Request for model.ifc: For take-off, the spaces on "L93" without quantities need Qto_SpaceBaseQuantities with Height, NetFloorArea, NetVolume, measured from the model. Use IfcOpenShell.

First a look at what the model holds.

```python
import ifcopenshell
import ifcopenshell.util.element
import ifcopenshell.util.unit

model = ifcopenshell.open("model.ifc")
print(model.schema)
for unit_type in ("LENGTHUNIT", "AREAUNIT", "VOLUMEUNIT"):
    print(unit_type, ifcopenshell.util.unit.calculate_unit_scale(model, unit_type))
storey = next(s for s in model.by_type("IfcBuildingStorey") if s.Name == "L93")
spaces = [e for e in ifcopenshell.util.element.get_decomposition(storey) if e.is_a("IfcSpace")]
for e in sorted(spaces, key=lambda e: e.id()):
    print(e.id(), e.is_a(), e.Name, list(ifcopenshell.util.element.get_psets(e, qtos_only=True)), sep=" | ")
```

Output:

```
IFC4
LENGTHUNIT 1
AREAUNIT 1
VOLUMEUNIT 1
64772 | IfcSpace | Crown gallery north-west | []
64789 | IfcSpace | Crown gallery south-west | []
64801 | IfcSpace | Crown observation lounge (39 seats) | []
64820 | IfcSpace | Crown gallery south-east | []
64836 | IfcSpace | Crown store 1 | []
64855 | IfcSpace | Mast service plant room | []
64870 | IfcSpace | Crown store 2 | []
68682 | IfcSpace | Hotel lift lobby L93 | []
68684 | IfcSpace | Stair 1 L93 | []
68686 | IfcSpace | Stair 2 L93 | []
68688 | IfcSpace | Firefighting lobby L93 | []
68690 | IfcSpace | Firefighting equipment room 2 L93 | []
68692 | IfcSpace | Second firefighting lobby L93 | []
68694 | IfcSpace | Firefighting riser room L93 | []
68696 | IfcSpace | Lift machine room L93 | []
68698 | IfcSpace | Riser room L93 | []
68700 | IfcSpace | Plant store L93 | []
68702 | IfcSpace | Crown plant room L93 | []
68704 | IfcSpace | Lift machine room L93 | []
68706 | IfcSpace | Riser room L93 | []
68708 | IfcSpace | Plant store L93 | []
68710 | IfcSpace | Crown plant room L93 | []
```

```python
import ifcopenshell
import ifcopenshell.api.pset
import ifcopenshell.geom
import ifcopenshell.util.element
import ifcopenshell.util.shape
import ifcopenshell.util.unit

model = ifcopenshell.open("model.ifc")
unit_scale = ifcopenshell.util.unit.calculate_unit_scale(model)
area_scale = ifcopenshell.util.unit.calculate_unit_scale(model, "AREAUNIT")
volume_scale = ifcopenshell.util.unit.calculate_unit_scale(model, "VOLUMEUNIT")
settings = ifcopenshell.geom.settings()

storey = next(s for s in model.by_type("IfcBuildingStorey") if s.Name == "L93")
spaces = [e for e in ifcopenshell.util.element.get_decomposition(storey) if e.is_a("IfcSpace")]

for e in sorted(spaces, key=lambda e: e.id()):
    if ifcopenshell.util.element.get_psets(e, qtos_only=True, should_inherit=False):
        continue
    # Geometry comes back in metres, in the element's own axes.
    shape = ifcopenshell.geom.create_shape(settings, e)
    values = {
        "Height": ifcopenshell.util.shape.get_z(shape.geometry) / unit_scale,
        "NetFloorArea": ifcopenshell.util.shape.get_footprint_area(shape.geometry) / area_scale,
        "NetVolume": ifcopenshell.util.shape.get_volume(shape.geometry) / volume_scale,
    }
    qto = ifcopenshell.api.pset.add_qto(model, product=e, name="Qto_SpaceBaseQuantities")
    ifcopenshell.api.pset.edit_qto(model, qto=qto, properties=values)
    print(e.id(), {k: round(v, 3) for k, v in values.items()})

model.write("model-out.ifc")
```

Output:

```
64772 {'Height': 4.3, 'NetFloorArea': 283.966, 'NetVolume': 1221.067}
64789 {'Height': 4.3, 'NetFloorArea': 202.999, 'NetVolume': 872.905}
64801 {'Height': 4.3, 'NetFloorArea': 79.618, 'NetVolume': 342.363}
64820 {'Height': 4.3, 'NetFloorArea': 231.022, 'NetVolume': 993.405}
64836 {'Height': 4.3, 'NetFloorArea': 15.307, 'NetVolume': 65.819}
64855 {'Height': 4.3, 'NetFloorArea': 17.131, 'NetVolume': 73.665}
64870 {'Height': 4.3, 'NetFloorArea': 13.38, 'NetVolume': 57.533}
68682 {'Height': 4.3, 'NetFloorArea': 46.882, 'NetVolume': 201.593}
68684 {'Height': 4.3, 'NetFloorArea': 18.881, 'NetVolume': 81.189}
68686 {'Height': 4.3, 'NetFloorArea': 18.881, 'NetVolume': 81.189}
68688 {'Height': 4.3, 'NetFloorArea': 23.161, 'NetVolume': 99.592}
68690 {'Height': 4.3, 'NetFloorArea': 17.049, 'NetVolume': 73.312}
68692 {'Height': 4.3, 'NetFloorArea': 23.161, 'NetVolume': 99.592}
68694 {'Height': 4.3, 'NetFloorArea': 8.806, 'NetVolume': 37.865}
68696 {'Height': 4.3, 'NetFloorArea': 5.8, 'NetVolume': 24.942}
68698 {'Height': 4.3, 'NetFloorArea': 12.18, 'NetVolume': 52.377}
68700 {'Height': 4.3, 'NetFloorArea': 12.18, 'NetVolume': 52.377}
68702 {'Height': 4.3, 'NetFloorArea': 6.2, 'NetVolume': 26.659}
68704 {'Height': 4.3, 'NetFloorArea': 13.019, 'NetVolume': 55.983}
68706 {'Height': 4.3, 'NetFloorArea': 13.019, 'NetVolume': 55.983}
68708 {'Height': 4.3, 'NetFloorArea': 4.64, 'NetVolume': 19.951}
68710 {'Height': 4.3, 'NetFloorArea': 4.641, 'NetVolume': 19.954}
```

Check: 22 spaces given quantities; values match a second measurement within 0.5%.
